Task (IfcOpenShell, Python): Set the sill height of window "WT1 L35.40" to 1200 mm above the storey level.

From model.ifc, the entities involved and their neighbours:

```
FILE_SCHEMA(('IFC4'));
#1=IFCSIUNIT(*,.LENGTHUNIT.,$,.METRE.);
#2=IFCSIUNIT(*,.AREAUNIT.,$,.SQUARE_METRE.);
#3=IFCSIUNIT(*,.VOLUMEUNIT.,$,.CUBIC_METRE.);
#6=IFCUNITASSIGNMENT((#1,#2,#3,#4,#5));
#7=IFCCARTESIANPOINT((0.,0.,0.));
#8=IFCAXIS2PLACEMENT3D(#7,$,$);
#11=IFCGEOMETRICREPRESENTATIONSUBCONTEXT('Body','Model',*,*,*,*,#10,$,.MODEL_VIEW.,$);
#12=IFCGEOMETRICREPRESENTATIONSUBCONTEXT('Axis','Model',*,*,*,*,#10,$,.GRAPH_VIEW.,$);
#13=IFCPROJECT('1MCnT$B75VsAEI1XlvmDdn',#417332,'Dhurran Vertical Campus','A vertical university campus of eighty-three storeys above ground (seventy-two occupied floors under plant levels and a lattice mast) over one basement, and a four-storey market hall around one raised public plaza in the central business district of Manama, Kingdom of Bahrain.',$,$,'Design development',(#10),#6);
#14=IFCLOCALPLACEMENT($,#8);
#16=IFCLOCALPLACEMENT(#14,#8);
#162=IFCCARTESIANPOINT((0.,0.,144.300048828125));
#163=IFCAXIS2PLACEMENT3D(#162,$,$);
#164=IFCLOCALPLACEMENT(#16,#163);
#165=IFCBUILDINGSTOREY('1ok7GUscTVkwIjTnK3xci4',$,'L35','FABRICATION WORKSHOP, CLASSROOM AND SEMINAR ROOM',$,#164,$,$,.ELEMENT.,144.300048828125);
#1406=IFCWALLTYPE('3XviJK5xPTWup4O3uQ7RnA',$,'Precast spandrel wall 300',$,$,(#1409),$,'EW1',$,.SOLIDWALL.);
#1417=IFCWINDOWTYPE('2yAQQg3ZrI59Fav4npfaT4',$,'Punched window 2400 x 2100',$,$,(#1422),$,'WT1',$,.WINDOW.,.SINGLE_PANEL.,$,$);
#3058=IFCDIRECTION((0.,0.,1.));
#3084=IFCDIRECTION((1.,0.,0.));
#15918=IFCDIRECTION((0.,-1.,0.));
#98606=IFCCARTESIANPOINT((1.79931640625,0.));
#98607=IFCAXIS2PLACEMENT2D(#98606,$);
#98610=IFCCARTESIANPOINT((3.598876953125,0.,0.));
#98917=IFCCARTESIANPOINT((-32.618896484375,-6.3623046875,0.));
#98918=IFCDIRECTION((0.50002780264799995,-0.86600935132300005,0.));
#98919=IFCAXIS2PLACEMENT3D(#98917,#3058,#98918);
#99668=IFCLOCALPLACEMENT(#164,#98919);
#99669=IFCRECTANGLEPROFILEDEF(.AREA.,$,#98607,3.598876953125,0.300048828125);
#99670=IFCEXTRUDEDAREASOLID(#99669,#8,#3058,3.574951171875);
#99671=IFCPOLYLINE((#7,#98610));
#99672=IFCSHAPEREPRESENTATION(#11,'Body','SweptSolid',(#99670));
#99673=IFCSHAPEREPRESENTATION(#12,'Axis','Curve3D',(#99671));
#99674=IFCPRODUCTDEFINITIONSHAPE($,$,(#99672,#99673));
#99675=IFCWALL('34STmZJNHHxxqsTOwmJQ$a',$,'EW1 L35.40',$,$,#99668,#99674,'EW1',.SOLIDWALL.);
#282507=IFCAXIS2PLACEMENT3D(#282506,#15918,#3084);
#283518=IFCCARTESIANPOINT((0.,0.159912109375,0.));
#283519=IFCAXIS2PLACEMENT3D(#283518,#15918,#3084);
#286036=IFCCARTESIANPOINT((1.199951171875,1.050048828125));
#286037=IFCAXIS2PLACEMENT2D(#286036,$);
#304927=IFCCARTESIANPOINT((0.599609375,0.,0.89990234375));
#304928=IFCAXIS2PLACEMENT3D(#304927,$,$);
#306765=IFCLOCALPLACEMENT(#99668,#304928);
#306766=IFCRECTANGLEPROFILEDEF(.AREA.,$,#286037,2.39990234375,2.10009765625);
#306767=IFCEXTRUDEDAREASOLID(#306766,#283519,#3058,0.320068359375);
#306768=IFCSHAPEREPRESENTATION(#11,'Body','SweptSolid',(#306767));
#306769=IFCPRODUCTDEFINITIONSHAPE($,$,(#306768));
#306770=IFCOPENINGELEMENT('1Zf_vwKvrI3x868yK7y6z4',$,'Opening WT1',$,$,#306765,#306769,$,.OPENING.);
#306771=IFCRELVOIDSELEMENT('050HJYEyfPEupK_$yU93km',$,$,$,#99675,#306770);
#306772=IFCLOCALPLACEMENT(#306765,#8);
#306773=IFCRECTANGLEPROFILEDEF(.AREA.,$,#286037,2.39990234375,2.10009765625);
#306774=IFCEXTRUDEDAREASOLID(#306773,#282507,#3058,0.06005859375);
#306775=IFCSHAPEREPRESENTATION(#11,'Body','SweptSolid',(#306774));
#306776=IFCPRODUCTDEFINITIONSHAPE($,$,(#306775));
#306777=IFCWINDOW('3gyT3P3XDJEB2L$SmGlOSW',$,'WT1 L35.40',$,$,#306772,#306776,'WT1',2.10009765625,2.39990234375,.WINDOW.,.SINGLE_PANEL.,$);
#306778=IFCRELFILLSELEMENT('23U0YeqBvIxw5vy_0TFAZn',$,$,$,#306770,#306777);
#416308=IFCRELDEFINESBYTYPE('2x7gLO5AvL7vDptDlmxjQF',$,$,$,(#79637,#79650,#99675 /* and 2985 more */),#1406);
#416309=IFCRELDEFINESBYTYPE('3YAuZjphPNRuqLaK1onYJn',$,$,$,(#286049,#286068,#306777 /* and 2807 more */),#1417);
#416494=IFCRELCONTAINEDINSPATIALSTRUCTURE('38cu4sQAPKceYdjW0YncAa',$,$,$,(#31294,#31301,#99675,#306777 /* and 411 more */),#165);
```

```python
import numpy as np
import ifcopenshell
import ifcopenshell.api.geometry
import ifcopenshell.geom
import ifcopenshell.util.element
import ifcopenshell.util.placement
import ifcopenshell.util.shape
import ifcopenshell.util.unit

model = ifcopenshell.open("model.ifc")
unit_scale = ifcopenshell.util.unit.calculate_unit_scale(model)

window = model.by_guid("3gyT3P3XDJEB2L$SmGlOSW")
opening = window.FillsVoids[0].RelatingOpeningElement
storey = ifcopenshell.util.element.get_container(window, ifc_class="IfcBuildingStorey")
level = ifcopenshell.util.placement.get_local_placement(storey.ObjectPlacement)[2, 3]

# The opening's origin need not be at the sill, so measure its lowest point.
shape = ifcopenshell.geom.create_shape(ifcopenshell.geom.settings(), opening)
bottom = ifcopenshell.util.shape.get_shape_bottom_elevation(shape, shape.geometry) / unit_scale
dz = level + 1.2 / unit_scale - bottom

shift = np.array([0.0, 0.0, dz])
# The window is placed relative to its opening, so it follows when the opening moves.
matrix = ifcopenshell.util.placement.get_local_placement(opening.ObjectPlacement)
matrix[:3, 3] += shift
ifcopenshell.api.geometry.edit_object_placement(
    model, product=opening, matrix=matrix, is_si=False, should_transform_children=True
)

print(f"moved by {dz * unit_scale:+.3f} m")

model.write("model_edited.ifc")
```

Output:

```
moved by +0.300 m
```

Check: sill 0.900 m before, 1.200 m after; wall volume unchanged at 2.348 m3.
